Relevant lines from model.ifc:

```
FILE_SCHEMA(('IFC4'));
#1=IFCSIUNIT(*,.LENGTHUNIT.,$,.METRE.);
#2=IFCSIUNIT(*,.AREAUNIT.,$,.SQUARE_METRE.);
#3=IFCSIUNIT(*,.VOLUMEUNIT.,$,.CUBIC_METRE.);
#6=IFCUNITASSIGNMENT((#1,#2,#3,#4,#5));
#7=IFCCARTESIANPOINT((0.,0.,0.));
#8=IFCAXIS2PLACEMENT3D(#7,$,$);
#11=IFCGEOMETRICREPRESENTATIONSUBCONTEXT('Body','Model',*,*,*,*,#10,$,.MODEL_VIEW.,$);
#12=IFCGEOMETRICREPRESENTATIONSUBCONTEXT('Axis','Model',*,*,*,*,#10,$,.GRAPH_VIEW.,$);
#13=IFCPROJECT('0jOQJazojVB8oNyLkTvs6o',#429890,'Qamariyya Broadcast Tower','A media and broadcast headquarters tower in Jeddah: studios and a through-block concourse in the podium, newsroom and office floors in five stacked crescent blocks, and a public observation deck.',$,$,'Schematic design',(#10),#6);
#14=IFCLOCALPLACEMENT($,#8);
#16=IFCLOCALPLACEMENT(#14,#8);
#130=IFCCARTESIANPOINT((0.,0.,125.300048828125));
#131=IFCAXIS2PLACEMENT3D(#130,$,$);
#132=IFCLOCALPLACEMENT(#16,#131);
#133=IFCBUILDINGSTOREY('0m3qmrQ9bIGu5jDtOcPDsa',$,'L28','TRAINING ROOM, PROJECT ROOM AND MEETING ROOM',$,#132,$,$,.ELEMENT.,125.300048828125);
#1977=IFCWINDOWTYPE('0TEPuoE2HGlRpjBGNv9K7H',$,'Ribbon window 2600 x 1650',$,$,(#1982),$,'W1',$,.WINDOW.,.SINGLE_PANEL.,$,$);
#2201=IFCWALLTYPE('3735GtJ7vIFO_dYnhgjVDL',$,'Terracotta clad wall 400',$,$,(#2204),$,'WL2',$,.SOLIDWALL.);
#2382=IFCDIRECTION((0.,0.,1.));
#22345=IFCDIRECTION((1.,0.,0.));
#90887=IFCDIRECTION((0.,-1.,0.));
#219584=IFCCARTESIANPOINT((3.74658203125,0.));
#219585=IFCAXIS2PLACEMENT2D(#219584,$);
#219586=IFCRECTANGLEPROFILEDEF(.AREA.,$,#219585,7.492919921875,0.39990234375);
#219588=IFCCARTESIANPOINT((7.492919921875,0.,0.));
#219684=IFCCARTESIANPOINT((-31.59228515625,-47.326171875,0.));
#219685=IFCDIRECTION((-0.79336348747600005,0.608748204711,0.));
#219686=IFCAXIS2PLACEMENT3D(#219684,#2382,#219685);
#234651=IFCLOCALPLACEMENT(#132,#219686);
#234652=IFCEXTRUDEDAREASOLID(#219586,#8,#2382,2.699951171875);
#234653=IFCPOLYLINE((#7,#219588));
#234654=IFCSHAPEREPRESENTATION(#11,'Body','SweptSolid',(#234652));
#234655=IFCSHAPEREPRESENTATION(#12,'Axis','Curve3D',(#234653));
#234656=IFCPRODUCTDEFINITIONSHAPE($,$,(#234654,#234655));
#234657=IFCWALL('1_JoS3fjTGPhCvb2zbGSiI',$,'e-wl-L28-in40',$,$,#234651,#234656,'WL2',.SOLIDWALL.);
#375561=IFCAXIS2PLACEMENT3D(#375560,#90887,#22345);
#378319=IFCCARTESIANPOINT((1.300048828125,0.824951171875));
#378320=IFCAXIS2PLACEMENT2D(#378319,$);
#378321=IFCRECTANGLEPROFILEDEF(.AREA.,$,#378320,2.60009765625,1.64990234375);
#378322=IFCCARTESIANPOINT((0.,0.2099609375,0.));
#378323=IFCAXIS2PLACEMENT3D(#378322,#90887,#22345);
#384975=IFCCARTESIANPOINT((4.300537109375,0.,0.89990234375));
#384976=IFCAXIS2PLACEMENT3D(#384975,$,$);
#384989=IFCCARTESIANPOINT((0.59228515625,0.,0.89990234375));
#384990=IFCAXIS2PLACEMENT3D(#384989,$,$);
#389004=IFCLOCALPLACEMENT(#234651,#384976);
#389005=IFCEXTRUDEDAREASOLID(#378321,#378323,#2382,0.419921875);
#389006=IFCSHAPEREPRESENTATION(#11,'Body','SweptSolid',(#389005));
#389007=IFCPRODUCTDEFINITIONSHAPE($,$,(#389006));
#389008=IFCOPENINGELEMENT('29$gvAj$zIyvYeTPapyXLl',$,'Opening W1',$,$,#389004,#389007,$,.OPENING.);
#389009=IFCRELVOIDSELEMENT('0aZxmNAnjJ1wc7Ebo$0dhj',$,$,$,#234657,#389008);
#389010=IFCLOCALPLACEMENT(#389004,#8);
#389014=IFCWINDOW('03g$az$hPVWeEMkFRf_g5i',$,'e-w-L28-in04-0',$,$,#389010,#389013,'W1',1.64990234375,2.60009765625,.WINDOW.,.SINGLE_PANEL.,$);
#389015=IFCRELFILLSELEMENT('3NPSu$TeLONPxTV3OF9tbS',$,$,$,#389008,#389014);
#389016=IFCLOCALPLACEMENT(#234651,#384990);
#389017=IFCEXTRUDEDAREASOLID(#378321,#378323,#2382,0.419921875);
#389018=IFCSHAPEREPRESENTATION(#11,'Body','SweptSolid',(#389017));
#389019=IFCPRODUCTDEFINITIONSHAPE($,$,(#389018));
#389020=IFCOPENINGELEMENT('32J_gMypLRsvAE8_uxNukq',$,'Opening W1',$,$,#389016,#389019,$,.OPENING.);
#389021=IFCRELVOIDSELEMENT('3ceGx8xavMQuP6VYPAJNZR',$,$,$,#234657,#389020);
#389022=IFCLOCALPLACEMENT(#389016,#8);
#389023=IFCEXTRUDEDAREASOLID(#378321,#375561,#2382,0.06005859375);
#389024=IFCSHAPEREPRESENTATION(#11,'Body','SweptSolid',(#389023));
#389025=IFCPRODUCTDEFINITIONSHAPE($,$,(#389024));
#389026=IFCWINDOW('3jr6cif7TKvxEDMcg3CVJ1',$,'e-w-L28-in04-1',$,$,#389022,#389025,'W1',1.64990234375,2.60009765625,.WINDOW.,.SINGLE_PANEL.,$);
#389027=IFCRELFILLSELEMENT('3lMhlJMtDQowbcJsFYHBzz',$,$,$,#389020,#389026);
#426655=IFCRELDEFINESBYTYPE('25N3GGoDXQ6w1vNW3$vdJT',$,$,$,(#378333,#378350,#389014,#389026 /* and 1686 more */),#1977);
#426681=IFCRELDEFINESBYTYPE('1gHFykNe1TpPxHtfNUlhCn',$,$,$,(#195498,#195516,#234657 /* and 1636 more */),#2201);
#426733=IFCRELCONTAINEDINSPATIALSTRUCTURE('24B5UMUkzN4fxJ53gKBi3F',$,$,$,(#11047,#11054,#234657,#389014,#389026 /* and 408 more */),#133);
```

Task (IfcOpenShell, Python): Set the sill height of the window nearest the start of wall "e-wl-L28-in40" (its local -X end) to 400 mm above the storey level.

```python
import numpy as np
import ifcopenshell
import ifcopenshell.api.geometry
import ifcopenshell.geom
import ifcopenshell.util.element
import ifcopenshell.util.placement
import ifcopenshell.util.shape
import ifcopenshell.util.unit

model = ifcopenshell.open("model.ifc")
unit_scale = ifcopenshell.util.unit.calculate_unit_scale(model)

window = model.by_guid("3jr6cif7TKvxEDMcg3CVJ1")
opening = window.FillsVoids[0].RelatingOpeningElement
storey = ifcopenshell.util.element.get_container(window, ifc_class="IfcBuildingStorey")
level = ifcopenshell.util.placement.get_local_placement(storey.ObjectPlacement)[2, 3]

# The opening's origin need not be at the sill, so measure its lowest point.
shape = ifcopenshell.geom.create_shape(ifcopenshell.geom.settings(), opening)
bottom = ifcopenshell.util.shape.get_shape_bottom_elevation(shape, shape.geometry) / unit_scale
dz = level + 0.4 - bottom

shift = np.array([0.0, 0.0, dz])
# The window is placed relative to its opening, so it follows when the opening moves.
matrix = ifcopenshell.util.placement.get_local_placement(opening.ObjectPlacement)
matrix[:3, 3] += shift
ifcopenshell.api.geometry.edit_object_placement(
    model, product=opening, matrix=matrix, is_si=False, should_transform_children=True
)

print(f"moved by {dz * unit_scale:+.3f} m")

model.write("model_edited.ifc")
```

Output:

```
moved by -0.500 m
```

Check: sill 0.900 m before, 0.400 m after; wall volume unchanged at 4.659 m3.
